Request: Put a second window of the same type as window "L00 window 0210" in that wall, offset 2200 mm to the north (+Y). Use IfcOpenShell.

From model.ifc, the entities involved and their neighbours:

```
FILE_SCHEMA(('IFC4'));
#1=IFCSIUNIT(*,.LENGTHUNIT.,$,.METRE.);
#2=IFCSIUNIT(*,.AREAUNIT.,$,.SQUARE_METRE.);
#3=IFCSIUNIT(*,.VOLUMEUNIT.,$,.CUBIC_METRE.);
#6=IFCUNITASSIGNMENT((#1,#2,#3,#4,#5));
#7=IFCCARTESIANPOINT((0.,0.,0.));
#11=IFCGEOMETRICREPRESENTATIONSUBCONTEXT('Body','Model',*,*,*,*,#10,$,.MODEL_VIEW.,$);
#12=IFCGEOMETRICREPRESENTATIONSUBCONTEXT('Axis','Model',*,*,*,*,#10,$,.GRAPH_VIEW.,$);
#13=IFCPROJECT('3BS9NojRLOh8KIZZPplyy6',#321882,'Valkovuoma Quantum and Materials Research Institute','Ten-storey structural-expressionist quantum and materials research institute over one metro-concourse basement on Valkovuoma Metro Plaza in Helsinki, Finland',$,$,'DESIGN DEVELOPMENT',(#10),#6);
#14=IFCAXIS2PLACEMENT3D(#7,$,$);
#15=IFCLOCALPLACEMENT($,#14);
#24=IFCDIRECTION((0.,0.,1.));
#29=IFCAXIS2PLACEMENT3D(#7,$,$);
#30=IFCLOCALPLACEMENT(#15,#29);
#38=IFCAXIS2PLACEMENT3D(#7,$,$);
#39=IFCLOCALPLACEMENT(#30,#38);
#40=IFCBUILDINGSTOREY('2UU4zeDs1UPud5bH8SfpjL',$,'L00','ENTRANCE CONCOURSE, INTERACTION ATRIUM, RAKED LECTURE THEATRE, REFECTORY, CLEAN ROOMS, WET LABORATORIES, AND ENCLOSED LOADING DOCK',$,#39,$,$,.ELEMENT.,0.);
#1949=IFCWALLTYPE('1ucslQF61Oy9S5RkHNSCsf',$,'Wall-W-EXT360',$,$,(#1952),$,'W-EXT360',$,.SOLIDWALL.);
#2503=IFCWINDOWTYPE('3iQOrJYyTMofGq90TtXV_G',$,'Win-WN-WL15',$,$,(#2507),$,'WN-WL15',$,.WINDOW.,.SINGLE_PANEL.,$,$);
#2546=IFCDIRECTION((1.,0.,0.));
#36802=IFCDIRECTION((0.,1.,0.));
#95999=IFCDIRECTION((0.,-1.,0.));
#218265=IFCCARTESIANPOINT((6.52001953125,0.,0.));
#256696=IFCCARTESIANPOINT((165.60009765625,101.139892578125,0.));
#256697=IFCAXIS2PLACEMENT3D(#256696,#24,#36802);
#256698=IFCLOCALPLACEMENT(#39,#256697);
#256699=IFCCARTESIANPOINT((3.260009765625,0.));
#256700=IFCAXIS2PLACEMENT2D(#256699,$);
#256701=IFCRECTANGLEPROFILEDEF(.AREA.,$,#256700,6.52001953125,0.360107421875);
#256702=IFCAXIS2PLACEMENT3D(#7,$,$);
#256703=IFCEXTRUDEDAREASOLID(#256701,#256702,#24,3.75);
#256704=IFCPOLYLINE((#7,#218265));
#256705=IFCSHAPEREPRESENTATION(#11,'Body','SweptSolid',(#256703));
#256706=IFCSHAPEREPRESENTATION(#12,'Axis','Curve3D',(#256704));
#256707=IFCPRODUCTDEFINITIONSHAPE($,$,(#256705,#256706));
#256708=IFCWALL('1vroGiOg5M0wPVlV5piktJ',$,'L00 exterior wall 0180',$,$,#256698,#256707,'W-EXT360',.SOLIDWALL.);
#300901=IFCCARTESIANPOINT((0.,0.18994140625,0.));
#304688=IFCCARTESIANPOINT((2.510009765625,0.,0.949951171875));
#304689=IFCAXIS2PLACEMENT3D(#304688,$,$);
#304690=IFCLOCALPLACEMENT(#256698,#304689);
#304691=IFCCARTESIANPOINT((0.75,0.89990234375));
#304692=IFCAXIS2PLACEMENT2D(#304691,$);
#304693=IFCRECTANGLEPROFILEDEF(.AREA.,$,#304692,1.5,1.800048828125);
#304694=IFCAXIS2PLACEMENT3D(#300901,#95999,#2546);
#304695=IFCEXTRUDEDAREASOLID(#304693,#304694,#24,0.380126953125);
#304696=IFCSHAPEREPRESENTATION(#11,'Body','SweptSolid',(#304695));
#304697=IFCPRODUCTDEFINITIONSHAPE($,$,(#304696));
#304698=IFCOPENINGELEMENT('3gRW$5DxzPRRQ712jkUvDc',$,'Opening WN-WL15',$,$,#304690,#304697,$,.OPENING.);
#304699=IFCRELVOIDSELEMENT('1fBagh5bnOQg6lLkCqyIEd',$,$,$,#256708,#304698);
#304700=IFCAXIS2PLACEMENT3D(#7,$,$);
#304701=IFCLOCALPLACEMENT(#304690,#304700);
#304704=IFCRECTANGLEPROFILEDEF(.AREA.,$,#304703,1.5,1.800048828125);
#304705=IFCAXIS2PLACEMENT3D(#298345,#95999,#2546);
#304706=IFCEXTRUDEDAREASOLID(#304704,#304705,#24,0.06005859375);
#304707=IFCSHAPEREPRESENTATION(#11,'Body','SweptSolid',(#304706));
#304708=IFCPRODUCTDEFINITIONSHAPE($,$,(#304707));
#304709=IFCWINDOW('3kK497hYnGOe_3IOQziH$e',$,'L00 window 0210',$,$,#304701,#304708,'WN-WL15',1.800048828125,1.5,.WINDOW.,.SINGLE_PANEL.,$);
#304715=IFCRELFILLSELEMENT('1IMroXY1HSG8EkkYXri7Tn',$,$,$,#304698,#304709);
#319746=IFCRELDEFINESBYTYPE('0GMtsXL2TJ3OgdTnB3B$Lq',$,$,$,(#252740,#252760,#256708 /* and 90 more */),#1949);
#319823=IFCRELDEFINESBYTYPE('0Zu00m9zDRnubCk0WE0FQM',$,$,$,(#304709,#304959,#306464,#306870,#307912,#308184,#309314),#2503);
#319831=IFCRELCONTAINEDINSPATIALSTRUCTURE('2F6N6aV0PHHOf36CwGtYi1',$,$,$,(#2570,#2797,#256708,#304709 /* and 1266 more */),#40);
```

```python
import ifcopenshell
import ifcopenshell.api.feature
import ifcopenshell.api.geometry
import ifcopenshell.api.root
import ifcopenshell.geom
import ifcopenshell.util.element
import ifcopenshell.util.placement
import ifcopenshell.util.shape
import ifcopenshell.util.unit

model = ifcopenshell.open("model.ifc")
unit_scale = ifcopenshell.util.unit.calculate_unit_scale(model)
settings = ifcopenshell.geom.settings()


def volume(element):
    """Net volume in cubic metres, openings subtracted."""
    shape = ifcopenshell.geom.create_shape(settings, element)
    return ifcopenshell.util.shape.get_volume(shape.geometry)


window = model.by_guid("3kK497hYnGOe_3IOQziH$e")
opening = window.FillsVoids[0].RelatingOpeningElement
wall = opening.VoidsElements[0].RelatingBuildingElement
before = volume(wall)
shift = ifcopenshell.util.placement.get_local_placement(wall.ObjectPlacement)[:3, 0] * 2.2 / unit_scale

# copy_class copies the void relationship, type, container and properties, but no geometry.
new_opening = ifcopenshell.api.root.copy_class(model, product=opening)
new_opening.Representation = ifcopenshell.util.element.copy_deep(
    model, opening.Representation, exclude=["IfcGeometricRepresentationContext", "IfcRepresentationMap"]
)
new_window = ifcopenshell.api.root.copy_class(model, product=window)
new_window.Representation = ifcopenshell.util.element.copy_deep(
    model, window.Representation, exclude=["IfcGeometricRepresentationContext", "IfcRepresentationMap"]
)
new_window.Tag = None
ifcopenshell.api.feature.add_filling(model, opening=new_opening, element=new_window)

for old, new in ((opening, new_opening), (window, new_window)):
    matrix = ifcopenshell.util.placement.get_local_placement(old.ObjectPlacement)
    matrix[:3, 3] += shift
    ifcopenshell.api.geometry.edit_object_placement(model, product=new, matrix=matrix, is_si=False)

after = volume(wall)

print(f"wall volume {before:.3f} -> {after:.3f} m3")

model.write("model_edited.ifc")
```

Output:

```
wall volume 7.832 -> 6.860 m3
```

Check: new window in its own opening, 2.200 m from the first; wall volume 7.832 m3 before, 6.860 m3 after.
